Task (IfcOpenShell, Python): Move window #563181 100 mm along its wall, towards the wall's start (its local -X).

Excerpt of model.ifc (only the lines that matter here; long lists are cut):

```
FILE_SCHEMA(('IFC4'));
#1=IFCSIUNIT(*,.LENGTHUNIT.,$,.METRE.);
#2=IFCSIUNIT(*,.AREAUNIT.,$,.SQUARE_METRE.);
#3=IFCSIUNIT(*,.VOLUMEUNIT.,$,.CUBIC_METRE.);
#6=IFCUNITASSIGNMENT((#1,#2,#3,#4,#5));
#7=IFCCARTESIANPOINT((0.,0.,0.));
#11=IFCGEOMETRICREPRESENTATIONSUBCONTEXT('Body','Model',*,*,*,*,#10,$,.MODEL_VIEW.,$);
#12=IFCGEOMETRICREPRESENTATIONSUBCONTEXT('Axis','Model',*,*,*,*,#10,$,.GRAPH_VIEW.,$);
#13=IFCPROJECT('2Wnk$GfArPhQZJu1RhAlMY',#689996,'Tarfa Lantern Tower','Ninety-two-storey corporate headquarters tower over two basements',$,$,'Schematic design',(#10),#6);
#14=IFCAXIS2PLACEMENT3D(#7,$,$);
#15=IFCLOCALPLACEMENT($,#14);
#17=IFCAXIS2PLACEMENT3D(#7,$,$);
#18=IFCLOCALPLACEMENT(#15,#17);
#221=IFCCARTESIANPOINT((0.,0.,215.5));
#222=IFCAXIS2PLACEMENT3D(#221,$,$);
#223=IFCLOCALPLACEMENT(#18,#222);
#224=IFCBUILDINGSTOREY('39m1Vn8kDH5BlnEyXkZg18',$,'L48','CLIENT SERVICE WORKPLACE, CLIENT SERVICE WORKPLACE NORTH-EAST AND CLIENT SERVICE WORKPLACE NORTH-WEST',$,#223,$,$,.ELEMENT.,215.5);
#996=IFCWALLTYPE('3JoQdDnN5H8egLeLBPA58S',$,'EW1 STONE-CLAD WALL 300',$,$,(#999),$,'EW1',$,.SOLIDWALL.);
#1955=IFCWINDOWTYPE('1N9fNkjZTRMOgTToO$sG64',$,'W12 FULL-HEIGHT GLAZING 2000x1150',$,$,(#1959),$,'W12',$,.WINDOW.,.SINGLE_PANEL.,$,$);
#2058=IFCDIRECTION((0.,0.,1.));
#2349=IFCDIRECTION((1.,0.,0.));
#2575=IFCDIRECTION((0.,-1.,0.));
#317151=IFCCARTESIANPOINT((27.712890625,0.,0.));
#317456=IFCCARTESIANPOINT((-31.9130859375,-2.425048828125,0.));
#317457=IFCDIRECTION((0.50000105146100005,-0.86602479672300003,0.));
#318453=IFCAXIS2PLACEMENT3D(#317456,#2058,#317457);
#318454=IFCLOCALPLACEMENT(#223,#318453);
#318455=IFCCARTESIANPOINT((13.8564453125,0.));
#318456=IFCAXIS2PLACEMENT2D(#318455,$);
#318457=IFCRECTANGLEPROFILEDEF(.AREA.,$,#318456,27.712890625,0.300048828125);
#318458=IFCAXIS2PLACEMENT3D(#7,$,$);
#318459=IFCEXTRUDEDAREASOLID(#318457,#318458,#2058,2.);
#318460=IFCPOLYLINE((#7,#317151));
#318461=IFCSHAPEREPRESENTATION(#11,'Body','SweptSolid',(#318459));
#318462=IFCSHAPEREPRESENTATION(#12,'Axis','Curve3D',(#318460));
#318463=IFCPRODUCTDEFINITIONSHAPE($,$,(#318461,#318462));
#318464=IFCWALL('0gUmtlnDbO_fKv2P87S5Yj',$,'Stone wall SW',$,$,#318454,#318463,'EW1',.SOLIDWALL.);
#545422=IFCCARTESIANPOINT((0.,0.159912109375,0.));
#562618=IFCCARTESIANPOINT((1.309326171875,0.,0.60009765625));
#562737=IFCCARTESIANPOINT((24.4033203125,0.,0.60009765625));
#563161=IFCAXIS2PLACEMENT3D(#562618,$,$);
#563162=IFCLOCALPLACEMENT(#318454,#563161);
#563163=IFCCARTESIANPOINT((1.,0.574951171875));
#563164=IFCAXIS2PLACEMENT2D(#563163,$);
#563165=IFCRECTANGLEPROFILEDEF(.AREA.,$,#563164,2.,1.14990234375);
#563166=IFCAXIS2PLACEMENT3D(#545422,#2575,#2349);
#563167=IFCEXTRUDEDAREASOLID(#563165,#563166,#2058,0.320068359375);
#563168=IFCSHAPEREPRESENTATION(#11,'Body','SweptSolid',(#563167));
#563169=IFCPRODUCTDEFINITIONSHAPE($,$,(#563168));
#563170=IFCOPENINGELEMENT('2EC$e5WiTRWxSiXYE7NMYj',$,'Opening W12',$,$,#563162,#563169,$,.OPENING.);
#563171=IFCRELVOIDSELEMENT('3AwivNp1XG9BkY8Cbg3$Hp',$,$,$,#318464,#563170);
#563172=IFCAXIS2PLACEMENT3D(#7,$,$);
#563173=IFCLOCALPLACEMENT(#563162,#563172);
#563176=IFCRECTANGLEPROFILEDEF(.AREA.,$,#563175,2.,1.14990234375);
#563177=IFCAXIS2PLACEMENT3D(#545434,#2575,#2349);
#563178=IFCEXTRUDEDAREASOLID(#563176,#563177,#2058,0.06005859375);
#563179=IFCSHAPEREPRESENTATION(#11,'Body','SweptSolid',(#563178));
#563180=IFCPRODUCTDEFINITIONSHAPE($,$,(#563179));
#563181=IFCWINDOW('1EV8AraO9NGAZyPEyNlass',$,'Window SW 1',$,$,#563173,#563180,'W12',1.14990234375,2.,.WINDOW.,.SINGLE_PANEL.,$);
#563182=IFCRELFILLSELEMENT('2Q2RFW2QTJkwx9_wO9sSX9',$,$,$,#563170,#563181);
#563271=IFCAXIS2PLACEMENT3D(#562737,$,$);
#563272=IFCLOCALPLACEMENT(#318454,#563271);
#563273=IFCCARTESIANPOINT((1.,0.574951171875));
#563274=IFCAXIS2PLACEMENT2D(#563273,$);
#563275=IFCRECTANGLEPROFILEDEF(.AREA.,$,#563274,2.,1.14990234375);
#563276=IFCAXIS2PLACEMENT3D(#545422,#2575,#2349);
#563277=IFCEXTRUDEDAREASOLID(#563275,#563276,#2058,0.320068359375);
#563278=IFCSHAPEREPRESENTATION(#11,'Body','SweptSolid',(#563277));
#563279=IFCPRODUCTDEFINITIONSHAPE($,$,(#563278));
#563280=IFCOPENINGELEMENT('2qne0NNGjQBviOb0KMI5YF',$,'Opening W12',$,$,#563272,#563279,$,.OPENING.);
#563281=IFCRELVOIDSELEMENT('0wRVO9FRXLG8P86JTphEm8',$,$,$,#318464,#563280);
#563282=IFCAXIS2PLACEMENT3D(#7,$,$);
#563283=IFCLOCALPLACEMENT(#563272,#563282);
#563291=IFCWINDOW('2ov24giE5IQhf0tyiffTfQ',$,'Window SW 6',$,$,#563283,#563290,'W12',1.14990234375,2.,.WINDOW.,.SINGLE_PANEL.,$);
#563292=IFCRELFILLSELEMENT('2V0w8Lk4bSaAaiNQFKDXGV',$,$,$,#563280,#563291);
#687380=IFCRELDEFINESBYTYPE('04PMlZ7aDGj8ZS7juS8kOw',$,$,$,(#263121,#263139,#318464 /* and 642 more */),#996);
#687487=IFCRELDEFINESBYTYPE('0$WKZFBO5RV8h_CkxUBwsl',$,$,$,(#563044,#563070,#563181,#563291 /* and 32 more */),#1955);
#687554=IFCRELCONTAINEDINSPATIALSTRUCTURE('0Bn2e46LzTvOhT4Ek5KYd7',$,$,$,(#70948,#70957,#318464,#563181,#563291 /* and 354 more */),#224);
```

```python
import ifcopenshell
import ifcopenshell.api.geometry
import ifcopenshell.util.placement

model = ifcopenshell.open("model.ifc")

window = model.by_id(563181)
opening = window.FillsVoids[0].RelatingOpeningElement
wall = opening.VoidsElements[0].RelatingBuildingElement

wall_matrix = ifcopenshell.util.placement.get_local_placement(wall.ObjectPlacement)
shift = wall_matrix[:3, 0] * -0.1
before = ifcopenshell.util.placement.get_local_placement(window.ObjectPlacement)[:3, 3].copy()

# The window is placed relative to its opening, so it follows when the opening moves.
matrix = ifcopenshell.util.placement.get_local_placement(opening.ObjectPlacement)
matrix[:3, 3] += shift
ifcopenshell.api.geometry.edit_object_placement(
    model, product=opening, matrix=matrix, is_si=False, should_transform_children=True
)

after = ifcopenshell.util.placement.get_local_placement(window.ObjectPlacement)[:3, 3]
print("window moved by", (after - before).round(3) + 0.0)

model.write("model_v2.ifc")
```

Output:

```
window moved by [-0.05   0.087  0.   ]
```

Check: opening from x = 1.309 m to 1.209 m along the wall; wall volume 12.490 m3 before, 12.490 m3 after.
